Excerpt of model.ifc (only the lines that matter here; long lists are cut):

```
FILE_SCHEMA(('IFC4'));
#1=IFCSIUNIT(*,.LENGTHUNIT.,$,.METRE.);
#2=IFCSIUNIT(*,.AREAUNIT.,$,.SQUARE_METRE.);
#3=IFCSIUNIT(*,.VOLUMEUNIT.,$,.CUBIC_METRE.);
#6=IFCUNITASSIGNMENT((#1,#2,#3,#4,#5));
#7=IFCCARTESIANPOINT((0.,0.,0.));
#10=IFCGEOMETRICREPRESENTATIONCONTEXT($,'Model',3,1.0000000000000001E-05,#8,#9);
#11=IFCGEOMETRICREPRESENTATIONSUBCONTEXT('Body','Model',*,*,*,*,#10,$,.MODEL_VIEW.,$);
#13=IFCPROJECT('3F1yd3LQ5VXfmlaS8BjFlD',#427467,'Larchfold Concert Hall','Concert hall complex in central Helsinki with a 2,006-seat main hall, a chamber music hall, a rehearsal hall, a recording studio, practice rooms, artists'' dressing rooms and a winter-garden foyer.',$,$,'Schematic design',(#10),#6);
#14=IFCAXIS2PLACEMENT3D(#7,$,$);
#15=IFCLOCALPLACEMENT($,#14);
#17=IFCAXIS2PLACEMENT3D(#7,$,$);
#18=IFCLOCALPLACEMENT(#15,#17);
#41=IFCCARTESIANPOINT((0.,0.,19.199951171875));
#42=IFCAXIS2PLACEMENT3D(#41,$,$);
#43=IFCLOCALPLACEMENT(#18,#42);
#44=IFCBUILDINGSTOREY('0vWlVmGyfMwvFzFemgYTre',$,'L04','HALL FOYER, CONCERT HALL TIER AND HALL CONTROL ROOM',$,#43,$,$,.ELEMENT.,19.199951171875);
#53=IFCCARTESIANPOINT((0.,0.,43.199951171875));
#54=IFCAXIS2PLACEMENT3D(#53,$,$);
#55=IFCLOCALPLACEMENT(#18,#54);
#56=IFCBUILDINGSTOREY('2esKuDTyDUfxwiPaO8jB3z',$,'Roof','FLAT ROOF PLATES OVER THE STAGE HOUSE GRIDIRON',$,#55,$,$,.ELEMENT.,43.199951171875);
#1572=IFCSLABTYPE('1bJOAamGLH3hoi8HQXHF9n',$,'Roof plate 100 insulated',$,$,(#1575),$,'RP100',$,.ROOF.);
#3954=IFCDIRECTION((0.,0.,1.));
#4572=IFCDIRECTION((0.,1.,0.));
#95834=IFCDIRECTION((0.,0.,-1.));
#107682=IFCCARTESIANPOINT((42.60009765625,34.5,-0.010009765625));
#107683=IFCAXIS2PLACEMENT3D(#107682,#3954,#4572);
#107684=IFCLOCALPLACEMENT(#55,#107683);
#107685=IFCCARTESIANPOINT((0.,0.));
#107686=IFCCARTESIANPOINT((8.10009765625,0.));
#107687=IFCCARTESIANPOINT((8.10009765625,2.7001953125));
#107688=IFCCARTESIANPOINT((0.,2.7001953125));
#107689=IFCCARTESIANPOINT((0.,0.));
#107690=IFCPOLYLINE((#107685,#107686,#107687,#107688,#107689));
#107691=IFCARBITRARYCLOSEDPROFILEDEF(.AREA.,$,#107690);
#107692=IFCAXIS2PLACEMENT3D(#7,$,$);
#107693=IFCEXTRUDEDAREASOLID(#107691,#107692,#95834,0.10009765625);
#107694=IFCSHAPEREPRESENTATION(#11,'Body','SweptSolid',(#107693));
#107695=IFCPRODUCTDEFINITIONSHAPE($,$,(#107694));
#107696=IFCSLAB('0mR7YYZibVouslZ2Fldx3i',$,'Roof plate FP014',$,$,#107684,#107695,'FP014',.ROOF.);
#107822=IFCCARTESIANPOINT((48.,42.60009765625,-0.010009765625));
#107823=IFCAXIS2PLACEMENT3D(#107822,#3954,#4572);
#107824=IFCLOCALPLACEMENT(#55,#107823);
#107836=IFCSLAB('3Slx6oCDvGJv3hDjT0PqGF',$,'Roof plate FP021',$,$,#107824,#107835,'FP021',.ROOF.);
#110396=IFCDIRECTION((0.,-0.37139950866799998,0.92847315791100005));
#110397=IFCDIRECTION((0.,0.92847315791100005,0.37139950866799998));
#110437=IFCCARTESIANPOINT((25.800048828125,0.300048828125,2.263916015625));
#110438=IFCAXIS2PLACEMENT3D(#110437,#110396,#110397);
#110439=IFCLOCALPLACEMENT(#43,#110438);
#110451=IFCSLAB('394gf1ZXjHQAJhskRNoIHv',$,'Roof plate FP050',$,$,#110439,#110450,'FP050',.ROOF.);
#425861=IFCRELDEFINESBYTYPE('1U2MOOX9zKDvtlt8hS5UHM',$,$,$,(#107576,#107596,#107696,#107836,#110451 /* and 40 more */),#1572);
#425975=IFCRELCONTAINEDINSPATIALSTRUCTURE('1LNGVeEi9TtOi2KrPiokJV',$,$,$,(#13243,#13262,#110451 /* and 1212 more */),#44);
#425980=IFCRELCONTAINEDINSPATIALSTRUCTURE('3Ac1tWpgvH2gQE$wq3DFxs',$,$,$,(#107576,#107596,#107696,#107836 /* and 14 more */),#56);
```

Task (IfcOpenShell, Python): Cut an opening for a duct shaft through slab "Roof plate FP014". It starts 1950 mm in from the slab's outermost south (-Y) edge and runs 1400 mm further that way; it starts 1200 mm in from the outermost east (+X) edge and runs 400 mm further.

```python
import numpy as np
import ifcopenshell
import ifcopenshell.api.feature
import ifcopenshell.api.geometry
import ifcopenshell.api.root
import ifcopenshell.geom
import ifcopenshell.util.placement
import ifcopenshell.util.representation
import ifcopenshell.util.shape
import ifcopenshell.util.unit

model = ifcopenshell.open("model.ifc")
unit_scale = ifcopenshell.util.unit.calculate_unit_scale(model)
settings = ifcopenshell.geom.settings()


def volume(element):
    """Net volume in cubic metres, openings subtracted."""
    shape = ifcopenshell.geom.create_shape(settings, element)
    return ifcopenshell.util.shape.get_volume(shape.geometry)


slab = model.by_id(107696)
before = volume(slab)

# Extent in the slab's own axes, in metres. The edges named are its -X and -Y sides.
slab_shape = ifcopenshell.geom.create_shape(settings, slab)
vertices = ifcopenshell.util.shape.get_vertices(slab_shape.geometry)
x_min, y_min, bottom = vertices.min(axis=0)
top = vertices[:, 2].max()

opening = ifcopenshell.api.root.create_entity(model, ifc_class="IfcOpeningElement", name="Duct shaft opening", predefined_type="OPENING")
context = ifcopenshell.util.representation.get_context(model, "Model", "Body", "MODEL_VIEW")
width, depth = 1.4, 0.4
outline = [(0.0, 0.0), (width, 0.0), (width, depth), (0.0, depth), (0.0, 0.0)]
# Overshoot both faces by 50 mm so the cut is clean.
shape = ifcopenshell.api.geometry.add_slab_representation(
    model, context=context, depth=top - bottom + 0.1, polyline=outline
)
ifcopenshell.api.geometry.assign_representation(model, product=opening, representation=shape)

matrix = ifcopenshell.util.placement.get_local_placement(slab.ObjectPlacement)
matrix[:, 3] = matrix @ np.append(np.array([x_min + 1.95, y_min + 1.2, bottom - 0.05]) / unit_scale, 1.0)
ifcopenshell.api.geometry.edit_object_placement(model, product=opening, matrix=matrix, is_si=False)
ifcopenshell.api.feature.add_feature(model, feature=opening, element=slab)

after = volume(slab)

print(f"slab volume {before:.3f} -> {after:.3f} m3")

model.write("model_edited.ifc")
```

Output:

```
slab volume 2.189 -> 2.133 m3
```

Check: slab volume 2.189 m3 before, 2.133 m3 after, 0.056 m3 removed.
